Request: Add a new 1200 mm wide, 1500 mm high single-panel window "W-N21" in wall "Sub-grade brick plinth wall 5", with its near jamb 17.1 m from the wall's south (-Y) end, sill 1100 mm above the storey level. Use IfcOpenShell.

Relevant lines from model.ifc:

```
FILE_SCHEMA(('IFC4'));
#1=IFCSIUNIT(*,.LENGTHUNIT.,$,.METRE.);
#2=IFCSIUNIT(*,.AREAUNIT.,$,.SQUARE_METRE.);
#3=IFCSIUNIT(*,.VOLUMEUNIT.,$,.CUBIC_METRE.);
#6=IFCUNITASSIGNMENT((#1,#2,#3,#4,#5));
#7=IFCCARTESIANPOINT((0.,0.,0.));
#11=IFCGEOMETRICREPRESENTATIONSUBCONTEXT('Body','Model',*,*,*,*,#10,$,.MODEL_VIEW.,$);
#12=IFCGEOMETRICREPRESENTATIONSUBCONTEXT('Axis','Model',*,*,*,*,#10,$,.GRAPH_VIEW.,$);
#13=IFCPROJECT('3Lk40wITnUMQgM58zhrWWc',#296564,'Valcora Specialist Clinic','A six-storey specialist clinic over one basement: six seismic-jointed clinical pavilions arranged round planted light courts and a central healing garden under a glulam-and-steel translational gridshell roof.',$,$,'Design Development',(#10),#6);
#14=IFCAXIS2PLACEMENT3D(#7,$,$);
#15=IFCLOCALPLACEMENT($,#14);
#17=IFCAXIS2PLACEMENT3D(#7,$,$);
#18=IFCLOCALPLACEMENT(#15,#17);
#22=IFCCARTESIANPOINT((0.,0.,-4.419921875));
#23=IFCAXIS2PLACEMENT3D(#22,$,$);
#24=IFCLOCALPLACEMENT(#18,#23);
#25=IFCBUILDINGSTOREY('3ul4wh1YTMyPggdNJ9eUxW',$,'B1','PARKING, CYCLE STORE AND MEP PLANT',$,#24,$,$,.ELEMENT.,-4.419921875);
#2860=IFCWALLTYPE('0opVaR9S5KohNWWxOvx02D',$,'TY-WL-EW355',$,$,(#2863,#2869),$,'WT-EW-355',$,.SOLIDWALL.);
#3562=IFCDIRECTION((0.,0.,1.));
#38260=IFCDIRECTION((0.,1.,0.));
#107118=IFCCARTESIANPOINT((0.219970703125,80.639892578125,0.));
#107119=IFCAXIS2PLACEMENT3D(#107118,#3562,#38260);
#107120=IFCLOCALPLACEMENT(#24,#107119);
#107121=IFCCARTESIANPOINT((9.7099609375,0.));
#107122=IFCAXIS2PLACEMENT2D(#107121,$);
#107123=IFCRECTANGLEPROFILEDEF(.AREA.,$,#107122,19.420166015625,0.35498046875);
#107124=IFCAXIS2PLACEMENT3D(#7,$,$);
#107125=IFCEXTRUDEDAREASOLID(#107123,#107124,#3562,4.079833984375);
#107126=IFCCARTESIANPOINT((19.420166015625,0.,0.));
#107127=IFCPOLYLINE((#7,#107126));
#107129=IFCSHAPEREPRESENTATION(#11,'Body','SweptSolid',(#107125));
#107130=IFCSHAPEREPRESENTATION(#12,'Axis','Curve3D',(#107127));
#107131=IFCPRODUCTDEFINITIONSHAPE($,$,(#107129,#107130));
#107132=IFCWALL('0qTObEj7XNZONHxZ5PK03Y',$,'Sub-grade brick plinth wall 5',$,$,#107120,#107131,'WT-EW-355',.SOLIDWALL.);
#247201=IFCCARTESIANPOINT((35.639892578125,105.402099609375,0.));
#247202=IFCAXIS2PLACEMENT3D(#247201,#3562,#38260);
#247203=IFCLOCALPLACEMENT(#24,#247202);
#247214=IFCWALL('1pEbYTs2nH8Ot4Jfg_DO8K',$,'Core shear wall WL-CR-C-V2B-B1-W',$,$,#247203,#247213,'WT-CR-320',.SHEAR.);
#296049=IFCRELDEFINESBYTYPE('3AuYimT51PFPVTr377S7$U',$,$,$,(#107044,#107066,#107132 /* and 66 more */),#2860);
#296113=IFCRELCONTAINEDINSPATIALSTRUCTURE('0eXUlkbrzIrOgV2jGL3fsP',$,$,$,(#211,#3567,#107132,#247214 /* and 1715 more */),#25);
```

```python
import numpy as np
import ifcopenshell
import ifcopenshell.api.feature
import ifcopenshell.api.geometry
import ifcopenshell.api.root
import ifcopenshell.api.spatial
import ifcopenshell.geom
import ifcopenshell.util.element
import ifcopenshell.util.placement
import ifcopenshell.util.representation
import ifcopenshell.util.shape
import ifcopenshell.util.unit

model = ifcopenshell.open("model.ifc")
unit_scale = ifcopenshell.util.unit.calculate_unit_scale(model)
settings = ifcopenshell.geom.settings()


def volume(element):
    """Net volume in cubic metres, openings subtracted."""
    shape = ifcopenshell.geom.create_shape(settings, element)
    return ifcopenshell.util.shape.get_volume(shape.geometry)


wall = model.by_guid("0qTObEj7XNZONHxZ5PK03Y")
storey = ifcopenshell.util.element.get_container(wall, ifc_class="IfcBuildingStorey")
context = ifcopenshell.util.representation.get_context(model, "Model", "Body", "MODEL_VIEW")
before = volume(wall)

width, height, from_end, sill = 1.2, 1.5, 17.1, 1.1  # metres

# The wall runs along its own X axis, and the end named is its -X end.
wall_shape = ifcopenshell.geom.create_shape(settings, wall)
x, y, z = ifcopenshell.util.shape.get_vertices(wall_shape.geometry).T
start = x.min() + from_end
face, thickness = float(y.min()), float(y.max() - y.min())
wall_matrix = ifcopenshell.util.placement.get_local_placement(wall.ObjectPlacement)
level = ifcopenshell.util.placement.get_local_placement(storey.ObjectPlacement)[2, 3]


def in_wall(x, y):
    """Placement at x, y metres in the wall's axes, at sill height."""
    matrix = wall_matrix.copy()
    matrix[:, 3] = wall_matrix @ np.array([x / unit_scale, y / unit_scale, 0.0, 1.0])
    matrix[2, 3] = level + sill / unit_scale
    return matrix


# Opening: a box that overshoots both wall faces by 50 mm.
opening = ifcopenshell.api.root.create_entity(model, ifc_class="IfcOpeningElement", predefined_type="OPENING")
box = ifcopenshell.api.geometry.add_wall_representation(
    model, context=context, length=width, height=height, thickness=thickness + 0.1
)
ifcopenshell.api.geometry.assign_representation(model, product=opening, representation=box)
ifcopenshell.api.geometry.edit_object_placement(model, product=opening, matrix=in_wall(start, face - 0.05), is_si=False)
ifcopenshell.api.feature.add_feature(model, feature=opening, element=wall)

window = ifcopenshell.api.root.create_entity(model, ifc_class="IfcWindow", name="W-N21", predefined_type="WINDOW")
window.OverallWidth, window.OverallHeight = width / unit_scale, height / unit_scale
window.PartitioningType = "SINGLE_PANEL"
body = ifcopenshell.api.geometry.add_window_representation(
    model,
    context=context,
    overall_width=window.OverallWidth,
    overall_height=window.OverallHeight,
    partition_type="SINGLE_PANEL",
)
ifcopenshell.api.geometry.assign_representation(model, product=window, representation=body)
ifcopenshell.api.spatial.assign_container(model, products=[window], relating_structure=storey)
ifcopenshell.api.feature.add_filling(model, opening=opening, element=window)

# Centre the window in the wall's thickness.
ifcopenshell.api.geometry.edit_object_placement(model, product=window, matrix=in_wall(start, face), is_si=False)
window_shape = ifcopenshell.geom.create_shape(settings, window)
depth = ifcopenshell.util.shape.get_vertices(window_shape.geometry)[:, 1]
offset = face + thickness / 2 - (depth.min() + depth.max()) / 2
ifcopenshell.api.geometry.edit_object_placement(model, product=window, matrix=in_wall(start, offset), is_si=False)

after = volume(wall)

print(f"wall volume {before:.3f} -> {after:.3f} m3")

model.write("model_rev.ifc")
```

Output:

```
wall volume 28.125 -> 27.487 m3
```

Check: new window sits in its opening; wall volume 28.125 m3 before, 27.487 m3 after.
